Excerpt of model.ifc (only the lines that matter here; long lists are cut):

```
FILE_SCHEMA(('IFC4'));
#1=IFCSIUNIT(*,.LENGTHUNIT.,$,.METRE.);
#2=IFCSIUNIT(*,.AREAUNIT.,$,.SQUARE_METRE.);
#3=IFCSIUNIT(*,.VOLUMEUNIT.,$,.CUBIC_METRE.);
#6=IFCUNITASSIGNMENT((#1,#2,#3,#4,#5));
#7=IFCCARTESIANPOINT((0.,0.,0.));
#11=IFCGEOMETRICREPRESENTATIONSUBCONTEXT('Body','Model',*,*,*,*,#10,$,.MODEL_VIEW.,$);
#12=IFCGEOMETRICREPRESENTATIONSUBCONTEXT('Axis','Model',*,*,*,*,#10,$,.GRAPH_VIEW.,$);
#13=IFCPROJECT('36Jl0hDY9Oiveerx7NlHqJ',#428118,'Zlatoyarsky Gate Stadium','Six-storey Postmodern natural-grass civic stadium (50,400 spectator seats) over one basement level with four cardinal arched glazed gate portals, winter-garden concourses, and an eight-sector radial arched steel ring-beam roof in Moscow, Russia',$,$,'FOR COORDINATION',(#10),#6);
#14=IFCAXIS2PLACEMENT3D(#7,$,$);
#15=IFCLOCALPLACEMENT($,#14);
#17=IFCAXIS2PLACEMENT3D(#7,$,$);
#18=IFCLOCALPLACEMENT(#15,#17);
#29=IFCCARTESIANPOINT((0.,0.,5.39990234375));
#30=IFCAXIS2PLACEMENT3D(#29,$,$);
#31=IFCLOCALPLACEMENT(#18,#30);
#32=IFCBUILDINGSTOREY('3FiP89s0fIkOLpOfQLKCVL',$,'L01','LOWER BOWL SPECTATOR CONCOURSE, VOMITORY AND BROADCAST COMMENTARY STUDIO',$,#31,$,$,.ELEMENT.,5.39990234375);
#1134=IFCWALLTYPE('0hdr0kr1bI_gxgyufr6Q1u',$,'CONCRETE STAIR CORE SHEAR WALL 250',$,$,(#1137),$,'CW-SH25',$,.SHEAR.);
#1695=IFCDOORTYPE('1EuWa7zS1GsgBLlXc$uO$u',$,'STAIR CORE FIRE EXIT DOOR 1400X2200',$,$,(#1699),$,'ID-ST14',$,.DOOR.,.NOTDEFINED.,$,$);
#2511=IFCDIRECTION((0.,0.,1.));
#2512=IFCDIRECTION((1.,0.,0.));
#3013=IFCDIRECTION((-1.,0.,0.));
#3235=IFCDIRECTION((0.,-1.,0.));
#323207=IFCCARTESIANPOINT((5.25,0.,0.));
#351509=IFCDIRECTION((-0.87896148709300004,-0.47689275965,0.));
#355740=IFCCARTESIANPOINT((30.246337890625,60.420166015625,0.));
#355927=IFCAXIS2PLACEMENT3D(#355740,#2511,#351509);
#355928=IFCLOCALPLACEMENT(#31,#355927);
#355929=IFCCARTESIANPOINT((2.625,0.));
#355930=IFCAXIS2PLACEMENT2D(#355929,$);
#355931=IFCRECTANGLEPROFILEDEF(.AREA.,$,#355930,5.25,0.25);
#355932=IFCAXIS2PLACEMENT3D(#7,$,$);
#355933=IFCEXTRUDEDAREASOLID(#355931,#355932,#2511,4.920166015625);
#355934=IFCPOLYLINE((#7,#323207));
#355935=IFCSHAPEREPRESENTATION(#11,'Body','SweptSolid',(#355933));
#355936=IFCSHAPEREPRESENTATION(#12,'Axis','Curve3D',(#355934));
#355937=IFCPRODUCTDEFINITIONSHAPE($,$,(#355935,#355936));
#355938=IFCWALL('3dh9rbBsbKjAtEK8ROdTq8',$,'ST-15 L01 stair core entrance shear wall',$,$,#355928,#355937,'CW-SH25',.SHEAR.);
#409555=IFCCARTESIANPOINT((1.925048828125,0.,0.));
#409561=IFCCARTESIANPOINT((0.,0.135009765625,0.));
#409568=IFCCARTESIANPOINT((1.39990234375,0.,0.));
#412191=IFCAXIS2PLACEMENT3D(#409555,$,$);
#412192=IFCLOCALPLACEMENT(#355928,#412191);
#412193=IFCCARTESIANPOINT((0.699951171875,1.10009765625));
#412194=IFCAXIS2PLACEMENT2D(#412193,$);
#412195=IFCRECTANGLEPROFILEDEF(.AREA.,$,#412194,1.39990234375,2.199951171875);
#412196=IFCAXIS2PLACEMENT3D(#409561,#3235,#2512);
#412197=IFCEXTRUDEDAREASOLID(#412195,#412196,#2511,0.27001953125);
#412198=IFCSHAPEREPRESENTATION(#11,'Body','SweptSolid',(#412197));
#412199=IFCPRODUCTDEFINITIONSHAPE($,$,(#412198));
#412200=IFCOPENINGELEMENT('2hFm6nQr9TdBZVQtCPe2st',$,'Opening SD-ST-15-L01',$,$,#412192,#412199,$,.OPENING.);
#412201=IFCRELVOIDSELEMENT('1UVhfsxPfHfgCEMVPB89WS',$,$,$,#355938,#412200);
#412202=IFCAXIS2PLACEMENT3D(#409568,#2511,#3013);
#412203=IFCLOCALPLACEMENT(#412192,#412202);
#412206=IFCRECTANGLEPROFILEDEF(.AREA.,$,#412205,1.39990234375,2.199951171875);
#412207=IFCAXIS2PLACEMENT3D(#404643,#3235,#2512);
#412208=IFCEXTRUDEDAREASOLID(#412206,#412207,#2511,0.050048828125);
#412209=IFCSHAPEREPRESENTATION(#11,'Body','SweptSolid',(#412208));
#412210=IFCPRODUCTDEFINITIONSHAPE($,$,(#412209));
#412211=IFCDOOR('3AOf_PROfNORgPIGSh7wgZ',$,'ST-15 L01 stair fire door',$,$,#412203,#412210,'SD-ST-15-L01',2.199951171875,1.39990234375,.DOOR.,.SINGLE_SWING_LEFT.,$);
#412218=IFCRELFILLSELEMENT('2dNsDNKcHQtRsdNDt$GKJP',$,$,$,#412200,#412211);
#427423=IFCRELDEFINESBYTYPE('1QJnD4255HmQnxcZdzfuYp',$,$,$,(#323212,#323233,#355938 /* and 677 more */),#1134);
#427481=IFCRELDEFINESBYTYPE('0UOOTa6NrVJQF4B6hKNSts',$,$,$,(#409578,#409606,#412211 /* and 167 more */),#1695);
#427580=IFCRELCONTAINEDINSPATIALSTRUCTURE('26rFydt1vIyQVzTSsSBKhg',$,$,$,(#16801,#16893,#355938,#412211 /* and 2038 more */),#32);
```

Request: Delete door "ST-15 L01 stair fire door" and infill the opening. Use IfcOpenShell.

```python
import ifcopenshell
import ifcopenshell.api.feature
import ifcopenshell.api.root
import ifcopenshell.geom
import ifcopenshell.util.shape

model = ifcopenshell.open("model.ifc")
settings = ifcopenshell.geom.settings()


def volume(element):
    """Net volume in cubic metres, openings subtracted."""
    shape = ifcopenshell.geom.create_shape(settings, element)
    return ifcopenshell.util.shape.get_volume(shape.geometry)


door = model.by_guid("3AOf_PROfNORgPIGSh7wgZ")
opening = door.FillsVoids[0].RelatingOpeningElement
wall = opening.VoidsElements[0].RelatingBuildingElement
before = volume(wall)

ifcopenshell.api.root.remove_product(model, product=door)
ifcopenshell.api.feature.remove_feature(model, feature=opening)

after = volume(wall)

print(f"wall volume {before:.3f} -> {after:.3f} m3")

model.write("model_rev.ifc")
```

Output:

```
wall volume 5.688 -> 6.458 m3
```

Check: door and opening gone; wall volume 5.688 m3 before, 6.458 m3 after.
